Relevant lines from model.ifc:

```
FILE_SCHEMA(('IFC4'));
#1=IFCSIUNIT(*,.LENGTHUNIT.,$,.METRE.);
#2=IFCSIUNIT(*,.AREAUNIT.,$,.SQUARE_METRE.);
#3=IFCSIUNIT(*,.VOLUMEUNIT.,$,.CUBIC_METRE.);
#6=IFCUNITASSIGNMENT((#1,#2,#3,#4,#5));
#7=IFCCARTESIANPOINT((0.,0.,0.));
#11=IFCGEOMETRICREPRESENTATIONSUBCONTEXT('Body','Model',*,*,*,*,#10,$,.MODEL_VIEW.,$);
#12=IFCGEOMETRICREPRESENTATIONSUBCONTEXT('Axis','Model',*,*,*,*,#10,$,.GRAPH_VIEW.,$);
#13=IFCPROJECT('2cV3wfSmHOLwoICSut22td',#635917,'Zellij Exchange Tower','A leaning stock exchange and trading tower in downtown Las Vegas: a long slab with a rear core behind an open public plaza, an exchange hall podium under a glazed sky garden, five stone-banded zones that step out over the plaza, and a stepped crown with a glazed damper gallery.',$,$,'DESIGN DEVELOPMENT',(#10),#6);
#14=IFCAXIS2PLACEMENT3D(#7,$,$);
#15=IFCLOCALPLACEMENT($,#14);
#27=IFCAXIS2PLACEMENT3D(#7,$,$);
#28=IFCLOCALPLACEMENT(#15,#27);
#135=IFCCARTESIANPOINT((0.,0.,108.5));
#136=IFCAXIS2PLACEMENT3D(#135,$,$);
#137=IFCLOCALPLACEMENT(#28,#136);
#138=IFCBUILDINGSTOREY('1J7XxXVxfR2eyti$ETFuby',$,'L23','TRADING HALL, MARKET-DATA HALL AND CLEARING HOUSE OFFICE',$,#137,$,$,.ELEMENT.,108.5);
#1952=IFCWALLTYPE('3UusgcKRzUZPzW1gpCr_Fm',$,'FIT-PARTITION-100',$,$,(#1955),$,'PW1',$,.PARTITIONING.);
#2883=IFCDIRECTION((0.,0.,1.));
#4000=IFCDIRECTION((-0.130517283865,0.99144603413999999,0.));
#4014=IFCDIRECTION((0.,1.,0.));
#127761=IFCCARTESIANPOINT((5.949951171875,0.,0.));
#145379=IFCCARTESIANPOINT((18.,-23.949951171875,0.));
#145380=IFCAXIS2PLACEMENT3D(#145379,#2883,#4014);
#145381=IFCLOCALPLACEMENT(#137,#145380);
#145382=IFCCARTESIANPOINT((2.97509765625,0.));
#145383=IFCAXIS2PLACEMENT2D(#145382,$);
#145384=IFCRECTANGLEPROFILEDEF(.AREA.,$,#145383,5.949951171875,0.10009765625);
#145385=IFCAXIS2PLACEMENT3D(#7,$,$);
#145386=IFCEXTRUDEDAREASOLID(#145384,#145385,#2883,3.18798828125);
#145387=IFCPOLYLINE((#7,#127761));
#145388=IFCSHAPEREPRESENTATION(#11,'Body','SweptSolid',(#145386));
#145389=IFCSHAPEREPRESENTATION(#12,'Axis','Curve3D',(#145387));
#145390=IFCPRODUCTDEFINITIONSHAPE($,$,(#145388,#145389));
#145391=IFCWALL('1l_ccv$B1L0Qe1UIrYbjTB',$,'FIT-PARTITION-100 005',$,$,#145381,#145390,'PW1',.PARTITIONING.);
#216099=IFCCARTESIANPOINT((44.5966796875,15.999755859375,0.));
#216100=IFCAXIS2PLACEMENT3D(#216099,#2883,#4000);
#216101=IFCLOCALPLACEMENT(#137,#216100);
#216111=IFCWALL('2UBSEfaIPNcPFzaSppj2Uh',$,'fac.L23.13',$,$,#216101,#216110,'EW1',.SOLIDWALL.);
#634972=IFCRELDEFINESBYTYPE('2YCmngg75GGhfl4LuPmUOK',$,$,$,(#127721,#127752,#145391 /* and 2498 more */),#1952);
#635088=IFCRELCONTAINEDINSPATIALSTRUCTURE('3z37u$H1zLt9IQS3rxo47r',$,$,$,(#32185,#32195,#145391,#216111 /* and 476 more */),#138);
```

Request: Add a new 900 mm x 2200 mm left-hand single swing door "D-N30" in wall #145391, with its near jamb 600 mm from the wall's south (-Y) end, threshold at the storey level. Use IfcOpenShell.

```python
import numpy as np
import ifcopenshell
import ifcopenshell.api.feature
import ifcopenshell.api.geometry
import ifcopenshell.api.root
import ifcopenshell.api.spatial
import ifcopenshell.geom
import ifcopenshell.util.element
import ifcopenshell.util.placement
import ifcopenshell.util.representation
import ifcopenshell.util.shape
import ifcopenshell.util.unit

model = ifcopenshell.open("model.ifc")
unit_scale = ifcopenshell.util.unit.calculate_unit_scale(model)
settings = ifcopenshell.geom.settings()


def volume(element):
    """Net volume in cubic metres, openings subtracted."""
    shape = ifcopenshell.geom.create_shape(settings, element)
    return ifcopenshell.util.shape.get_volume(shape.geometry)


wall = model.by_guid("1l_ccv$B1L0Qe1UIrYbjTB")
storey = ifcopenshell.util.element.get_container(wall, ifc_class="IfcBuildingStorey")
context = ifcopenshell.util.representation.get_context(model, "Model", "Body", "MODEL_VIEW")
before = volume(wall)

width, height, from_end, sill = 0.9, 2.2, 0.6, 0.0  # metres

# The wall runs along its own X axis, and the end named is its -X end.
wall_shape = ifcopenshell.geom.create_shape(settings, wall)
x, y, z = ifcopenshell.util.shape.get_vertices(wall_shape.geometry).T
start = x.min() + from_end
face, thickness = float(y.min()), float(y.max() - y.min())
wall_matrix = ifcopenshell.util.placement.get_local_placement(wall.ObjectPlacement)
level = ifcopenshell.util.placement.get_local_placement(storey.ObjectPlacement)[2, 3]


def in_wall(x, y):
    """Placement at x, y metres in the wall's axes, at sill height."""
    matrix = wall_matrix.copy()
    matrix[:, 3] = wall_matrix @ np.array([x / unit_scale, y / unit_scale, 0.0, 1.0])
    matrix[2, 3] = level + sill / unit_scale
    return matrix


# Opening: a box that overshoots both wall faces by 50 mm.
opening = ifcopenshell.api.root.create_entity(model, ifc_class="IfcOpeningElement", predefined_type="OPENING")
box = ifcopenshell.api.geometry.add_wall_representation(
    model, context=context, length=width, height=height, thickness=thickness + 0.1
)
ifcopenshell.api.geometry.assign_representation(model, product=opening, representation=box)
ifcopenshell.api.geometry.edit_object_placement(model, product=opening, matrix=in_wall(start, face - 0.05), is_si=False)
ifcopenshell.api.feature.add_feature(model, feature=opening, element=wall)

door = ifcopenshell.api.root.create_entity(model, ifc_class="IfcDoor", name="D-N30", predefined_type="DOOR")
door.OverallWidth, door.OverallHeight = width / unit_scale, height / unit_scale
door.OperationType = "SINGLE_SWING_LEFT"
body = ifcopenshell.api.geometry.add_door_representation(
    model,
    context=context,
    overall_width=door.OverallWidth,
    overall_height=door.OverallHeight,
    operation_type="SINGLE_SWING_LEFT",
    lining_properties={"LiningDepth": thickness / unit_scale, "ThresholdDepth": thickness / unit_scale},
)
ifcopenshell.api.geometry.assign_representation(model, product=door, representation=body)
ifcopenshell.api.spatial.assign_container(model, products=[door], relating_structure=storey)
ifcopenshell.api.feature.add_filling(model, opening=opening, element=door)

# The lining spans the wall, so the door starts at the wall face.
ifcopenshell.api.geometry.edit_object_placement(model, product=door, matrix=in_wall(start, face), is_si=False)

after = volume(wall)

print(f"wall volume {before:.3f} -> {after:.3f} m3")

model.write("model_edited.ifc")
```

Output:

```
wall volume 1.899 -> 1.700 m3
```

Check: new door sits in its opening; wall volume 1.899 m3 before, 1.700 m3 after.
